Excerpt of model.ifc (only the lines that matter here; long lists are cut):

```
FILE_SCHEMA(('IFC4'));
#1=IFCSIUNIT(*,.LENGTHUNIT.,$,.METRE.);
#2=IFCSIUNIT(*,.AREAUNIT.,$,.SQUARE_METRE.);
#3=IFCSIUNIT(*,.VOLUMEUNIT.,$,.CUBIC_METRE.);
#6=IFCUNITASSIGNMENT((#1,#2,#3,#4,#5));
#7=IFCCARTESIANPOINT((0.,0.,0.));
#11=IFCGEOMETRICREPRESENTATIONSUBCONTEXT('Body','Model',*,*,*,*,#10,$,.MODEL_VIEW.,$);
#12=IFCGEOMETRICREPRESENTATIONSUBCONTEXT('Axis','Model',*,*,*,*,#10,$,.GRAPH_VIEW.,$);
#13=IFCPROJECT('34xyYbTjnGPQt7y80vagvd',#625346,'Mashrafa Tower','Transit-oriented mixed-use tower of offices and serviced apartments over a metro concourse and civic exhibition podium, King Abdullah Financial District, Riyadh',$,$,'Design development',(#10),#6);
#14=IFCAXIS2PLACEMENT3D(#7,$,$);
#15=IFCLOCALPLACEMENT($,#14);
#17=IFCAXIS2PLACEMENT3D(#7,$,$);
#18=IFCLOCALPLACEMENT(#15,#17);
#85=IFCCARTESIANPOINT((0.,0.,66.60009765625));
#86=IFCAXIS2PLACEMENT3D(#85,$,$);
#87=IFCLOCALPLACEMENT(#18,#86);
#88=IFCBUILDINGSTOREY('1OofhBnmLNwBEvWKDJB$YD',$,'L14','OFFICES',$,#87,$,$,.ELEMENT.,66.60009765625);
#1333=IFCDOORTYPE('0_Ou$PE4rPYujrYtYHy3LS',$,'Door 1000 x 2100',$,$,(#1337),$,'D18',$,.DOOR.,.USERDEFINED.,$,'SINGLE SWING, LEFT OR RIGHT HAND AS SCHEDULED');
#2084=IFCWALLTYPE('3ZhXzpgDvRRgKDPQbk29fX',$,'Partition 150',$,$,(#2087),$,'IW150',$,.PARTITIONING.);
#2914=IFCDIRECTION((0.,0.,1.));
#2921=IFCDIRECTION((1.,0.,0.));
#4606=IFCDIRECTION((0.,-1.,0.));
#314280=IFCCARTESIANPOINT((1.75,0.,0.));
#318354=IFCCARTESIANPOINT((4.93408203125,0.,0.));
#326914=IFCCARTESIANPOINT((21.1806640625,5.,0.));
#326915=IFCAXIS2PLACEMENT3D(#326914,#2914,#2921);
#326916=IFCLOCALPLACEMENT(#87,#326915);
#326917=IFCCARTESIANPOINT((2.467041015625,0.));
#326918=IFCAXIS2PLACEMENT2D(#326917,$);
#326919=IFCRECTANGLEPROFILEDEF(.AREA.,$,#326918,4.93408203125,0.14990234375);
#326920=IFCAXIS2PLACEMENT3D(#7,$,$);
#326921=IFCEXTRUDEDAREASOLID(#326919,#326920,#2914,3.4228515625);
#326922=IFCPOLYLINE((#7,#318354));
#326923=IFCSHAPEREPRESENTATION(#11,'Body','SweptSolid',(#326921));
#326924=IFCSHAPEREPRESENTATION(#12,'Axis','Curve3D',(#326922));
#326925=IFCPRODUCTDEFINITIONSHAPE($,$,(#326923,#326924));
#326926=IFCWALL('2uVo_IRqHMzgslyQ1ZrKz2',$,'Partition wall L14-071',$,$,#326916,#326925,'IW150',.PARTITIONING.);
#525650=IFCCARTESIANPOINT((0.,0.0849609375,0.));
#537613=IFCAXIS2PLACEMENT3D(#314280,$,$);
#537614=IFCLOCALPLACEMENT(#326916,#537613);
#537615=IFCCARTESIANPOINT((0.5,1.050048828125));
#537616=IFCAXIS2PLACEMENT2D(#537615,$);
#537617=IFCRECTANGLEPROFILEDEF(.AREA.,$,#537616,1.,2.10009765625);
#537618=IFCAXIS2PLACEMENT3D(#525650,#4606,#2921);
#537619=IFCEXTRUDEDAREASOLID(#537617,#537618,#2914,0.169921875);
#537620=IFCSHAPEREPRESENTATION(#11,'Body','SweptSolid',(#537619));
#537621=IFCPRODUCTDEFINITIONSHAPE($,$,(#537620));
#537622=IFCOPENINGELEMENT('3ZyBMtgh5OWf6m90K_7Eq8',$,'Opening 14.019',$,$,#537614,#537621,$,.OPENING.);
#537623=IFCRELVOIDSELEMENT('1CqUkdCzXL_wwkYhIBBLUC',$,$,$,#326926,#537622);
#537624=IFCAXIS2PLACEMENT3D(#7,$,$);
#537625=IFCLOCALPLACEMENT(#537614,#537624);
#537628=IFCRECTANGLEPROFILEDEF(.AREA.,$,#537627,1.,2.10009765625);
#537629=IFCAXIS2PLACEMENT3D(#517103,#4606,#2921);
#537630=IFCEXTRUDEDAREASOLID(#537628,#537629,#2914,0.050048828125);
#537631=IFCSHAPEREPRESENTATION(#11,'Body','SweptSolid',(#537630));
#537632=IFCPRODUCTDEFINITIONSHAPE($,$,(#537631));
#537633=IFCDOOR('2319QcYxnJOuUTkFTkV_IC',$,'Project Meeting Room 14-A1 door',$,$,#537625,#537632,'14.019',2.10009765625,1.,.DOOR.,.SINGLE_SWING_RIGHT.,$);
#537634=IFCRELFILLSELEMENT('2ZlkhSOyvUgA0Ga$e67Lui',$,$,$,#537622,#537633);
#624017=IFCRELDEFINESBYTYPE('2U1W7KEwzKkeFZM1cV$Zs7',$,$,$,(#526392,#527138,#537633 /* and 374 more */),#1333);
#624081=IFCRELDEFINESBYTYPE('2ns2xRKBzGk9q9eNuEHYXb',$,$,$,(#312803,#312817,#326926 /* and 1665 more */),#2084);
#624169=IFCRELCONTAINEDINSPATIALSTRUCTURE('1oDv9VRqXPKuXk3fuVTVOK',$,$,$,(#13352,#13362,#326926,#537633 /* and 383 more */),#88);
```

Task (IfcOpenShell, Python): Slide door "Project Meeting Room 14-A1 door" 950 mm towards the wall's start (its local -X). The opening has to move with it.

```python
import ifcopenshell
import ifcopenshell.api.geometry
import ifcopenshell.util.placement
import ifcopenshell.util.unit

model = ifcopenshell.open("model.ifc")
unit_scale = ifcopenshell.util.unit.calculate_unit_scale(model)

door = model.by_guid("2319QcYxnJOuUTkFTkV_IC")
opening = door.FillsVoids[0].RelatingOpeningElement
wall = opening.VoidsElements[0].RelatingBuildingElement

wall_matrix = ifcopenshell.util.placement.get_local_placement(wall.ObjectPlacement)
shift = wall_matrix[:3, 0] * -0.95 / unit_scale
before = ifcopenshell.util.placement.get_local_placement(door.ObjectPlacement)[:3, 3].copy()

# The door is placed relative to its opening, so it follows when the opening moves.
matrix = ifcopenshell.util.placement.get_local_placement(opening.ObjectPlacement)
matrix[:3, 3] += shift
ifcopenshell.api.geometry.edit_object_placement(
    model, product=opening, matrix=matrix, is_si=False, should_transform_children=True
)

after = ifcopenshell.util.placement.get_local_placement(door.ObjectPlacement)[:3, 3]
print("door moved by", (after - before).round(3) + 0.0)

model.write("model_updated.ifc")
```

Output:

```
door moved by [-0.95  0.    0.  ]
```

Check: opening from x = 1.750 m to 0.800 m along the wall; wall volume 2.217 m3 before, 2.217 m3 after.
